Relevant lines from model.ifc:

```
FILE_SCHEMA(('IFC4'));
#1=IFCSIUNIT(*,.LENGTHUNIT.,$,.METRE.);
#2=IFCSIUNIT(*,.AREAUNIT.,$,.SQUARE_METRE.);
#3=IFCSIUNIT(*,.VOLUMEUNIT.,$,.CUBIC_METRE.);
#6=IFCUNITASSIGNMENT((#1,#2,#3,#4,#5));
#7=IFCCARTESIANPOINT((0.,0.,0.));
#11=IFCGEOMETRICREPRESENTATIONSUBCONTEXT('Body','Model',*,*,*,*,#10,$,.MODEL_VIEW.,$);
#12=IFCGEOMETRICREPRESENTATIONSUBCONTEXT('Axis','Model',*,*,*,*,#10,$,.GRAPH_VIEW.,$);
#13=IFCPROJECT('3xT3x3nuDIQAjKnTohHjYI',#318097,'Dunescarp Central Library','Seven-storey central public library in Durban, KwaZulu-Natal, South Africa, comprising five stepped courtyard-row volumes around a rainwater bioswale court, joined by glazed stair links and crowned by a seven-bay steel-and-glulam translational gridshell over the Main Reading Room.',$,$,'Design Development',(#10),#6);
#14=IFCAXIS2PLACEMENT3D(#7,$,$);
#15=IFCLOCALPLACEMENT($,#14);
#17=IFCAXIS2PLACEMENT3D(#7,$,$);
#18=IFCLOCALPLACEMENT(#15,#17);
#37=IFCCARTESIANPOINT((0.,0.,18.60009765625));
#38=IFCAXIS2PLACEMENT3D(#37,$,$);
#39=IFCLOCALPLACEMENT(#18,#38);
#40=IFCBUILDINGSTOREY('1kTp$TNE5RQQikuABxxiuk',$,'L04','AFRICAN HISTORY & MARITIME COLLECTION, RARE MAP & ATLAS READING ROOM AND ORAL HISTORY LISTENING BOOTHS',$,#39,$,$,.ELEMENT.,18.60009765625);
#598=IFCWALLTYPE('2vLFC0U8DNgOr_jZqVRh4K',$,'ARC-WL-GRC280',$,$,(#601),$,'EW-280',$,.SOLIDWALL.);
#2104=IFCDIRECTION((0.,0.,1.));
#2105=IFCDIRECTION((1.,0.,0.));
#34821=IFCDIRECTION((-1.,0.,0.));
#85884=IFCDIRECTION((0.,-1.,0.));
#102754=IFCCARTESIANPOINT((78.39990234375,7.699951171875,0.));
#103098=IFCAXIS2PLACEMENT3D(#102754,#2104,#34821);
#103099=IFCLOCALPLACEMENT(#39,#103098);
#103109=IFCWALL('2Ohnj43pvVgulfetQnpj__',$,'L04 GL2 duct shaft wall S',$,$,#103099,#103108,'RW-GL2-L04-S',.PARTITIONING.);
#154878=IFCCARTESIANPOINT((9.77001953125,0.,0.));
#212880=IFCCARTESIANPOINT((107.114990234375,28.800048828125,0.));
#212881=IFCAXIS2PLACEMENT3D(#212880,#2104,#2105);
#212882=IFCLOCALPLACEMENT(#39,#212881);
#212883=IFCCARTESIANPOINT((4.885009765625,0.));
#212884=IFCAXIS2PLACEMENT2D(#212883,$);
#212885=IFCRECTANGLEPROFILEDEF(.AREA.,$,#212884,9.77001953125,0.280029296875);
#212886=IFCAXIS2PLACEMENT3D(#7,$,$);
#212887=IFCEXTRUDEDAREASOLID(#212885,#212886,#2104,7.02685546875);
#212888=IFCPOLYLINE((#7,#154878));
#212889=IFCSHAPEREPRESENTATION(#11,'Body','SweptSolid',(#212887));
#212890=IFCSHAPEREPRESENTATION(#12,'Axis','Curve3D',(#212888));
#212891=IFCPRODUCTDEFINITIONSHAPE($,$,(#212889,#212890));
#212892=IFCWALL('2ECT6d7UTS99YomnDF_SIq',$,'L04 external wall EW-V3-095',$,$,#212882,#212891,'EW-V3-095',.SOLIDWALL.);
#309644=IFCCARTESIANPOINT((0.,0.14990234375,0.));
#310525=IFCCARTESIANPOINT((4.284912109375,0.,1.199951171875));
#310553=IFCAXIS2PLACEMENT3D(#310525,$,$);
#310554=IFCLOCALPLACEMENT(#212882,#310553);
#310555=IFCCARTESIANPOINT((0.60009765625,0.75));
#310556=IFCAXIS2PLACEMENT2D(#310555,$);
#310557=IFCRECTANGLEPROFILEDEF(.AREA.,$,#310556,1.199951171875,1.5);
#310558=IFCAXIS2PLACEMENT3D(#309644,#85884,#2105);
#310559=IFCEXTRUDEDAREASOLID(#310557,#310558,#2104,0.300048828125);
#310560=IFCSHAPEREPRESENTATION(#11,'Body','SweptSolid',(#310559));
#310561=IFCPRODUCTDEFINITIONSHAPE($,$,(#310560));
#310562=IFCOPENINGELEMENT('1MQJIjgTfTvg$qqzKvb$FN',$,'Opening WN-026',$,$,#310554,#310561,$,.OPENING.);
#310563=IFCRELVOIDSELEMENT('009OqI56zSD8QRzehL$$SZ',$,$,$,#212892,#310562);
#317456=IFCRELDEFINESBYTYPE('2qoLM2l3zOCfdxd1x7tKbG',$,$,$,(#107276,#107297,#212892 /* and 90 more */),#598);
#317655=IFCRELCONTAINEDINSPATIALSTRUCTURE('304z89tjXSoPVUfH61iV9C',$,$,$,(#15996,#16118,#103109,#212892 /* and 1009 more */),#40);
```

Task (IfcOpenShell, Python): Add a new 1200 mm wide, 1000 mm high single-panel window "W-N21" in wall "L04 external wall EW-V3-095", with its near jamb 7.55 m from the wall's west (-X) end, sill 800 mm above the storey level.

```python
import numpy as np
import ifcopenshell
import ifcopenshell.api.feature
import ifcopenshell.api.geometry
import ifcopenshell.api.root
import ifcopenshell.api.spatial
import ifcopenshell.geom
import ifcopenshell.util.element
import ifcopenshell.util.placement
import ifcopenshell.util.representation
import ifcopenshell.util.shape
import ifcopenshell.util.unit

model = ifcopenshell.open("model.ifc")
unit_scale = ifcopenshell.util.unit.calculate_unit_scale(model)
settings = ifcopenshell.geom.settings()


def volume(element):
    """Net volume in cubic metres, openings subtracted."""
    shape = ifcopenshell.geom.create_shape(settings, element)
    return ifcopenshell.util.shape.get_volume(shape.geometry)


wall = model.by_id(212892)
storey = ifcopenshell.util.element.get_container(wall, ifc_class="IfcBuildingStorey")
context = ifcopenshell.util.representation.get_context(model, "Model", "Body", "MODEL_VIEW")
before = volume(wall)

width, height, from_end, sill = 1.2, 1, 7.55, 0.8  # metres

# The wall runs along its own X axis, and the end named is its -X end.
wall_shape = ifcopenshell.geom.create_shape(settings, wall)
x, y, z = ifcopenshell.util.shape.get_vertices(wall_shape.geometry).T
start = x.min() + from_end
face, thickness = float(y.min()), float(y.max() - y.min())
wall_matrix = ifcopenshell.util.placement.get_local_placement(wall.ObjectPlacement)
level = ifcopenshell.util.placement.get_local_placement(storey.ObjectPlacement)[2, 3]


def in_wall(x, y):
    """Placement at x, y metres in the wall's axes, at sill height."""
    matrix = wall_matrix.copy()
    matrix[:, 3] = wall_matrix @ np.array([x / unit_scale, y / unit_scale, 0.0, 1.0])
    matrix[2, 3] = level + sill / unit_scale
    return matrix


# Opening: a box that overshoots both wall faces by 50 mm.
opening = ifcopenshell.api.root.create_entity(model, ifc_class="IfcOpeningElement", predefined_type="OPENING")
box = ifcopenshell.api.geometry.add_wall_representation(
    model, context=context, length=width, height=height, thickness=thickness + 0.1
)
ifcopenshell.api.geometry.assign_representation(model, product=opening, representation=box)
ifcopenshell.api.geometry.edit_object_placement(model, product=opening, matrix=in_wall(start, face - 0.05), is_si=False)
ifcopenshell.api.feature.add_feature(model, feature=opening, element=wall)

window = ifcopenshell.api.root.create_entity(model, ifc_class="IfcWindow", name="W-N21", predefined_type="WINDOW")
window.OverallWidth, window.OverallHeight = width / unit_scale, height / unit_scale
window.PartitioningType = "SINGLE_PANEL"
body = ifcopenshell.api.geometry.add_window_representation(
    model,
    context=context,
    overall_width=window.OverallWidth,
    overall_height=window.OverallHeight,
    partition_type="SINGLE_PANEL",
)
ifcopenshell.api.geometry.assign_representation(model, product=window, representation=body)
ifcopenshell.api.spatial.assign_container(model, products=[window], relating_structure=storey)
ifcopenshell.api.feature.add_filling(model, opening=opening, element=window)

# Centre the window in the wall's thickness.
ifcopenshell.api.geometry.edit_object_placement(model, product=window, matrix=in_wall(start, face), is_si=False)
window_shape = ifcopenshell.geom.create_shape(settings, window)
depth = ifcopenshell.util.shape.get_vertices(window_shape.geometry)[:, 1]
offset = face + thickness / 2 - (depth.min() + depth.max()) / 2
ifcopenshell.api.geometry.edit_object_placement(model, product=window, matrix=in_wall(start, offset), is_si=False)

after = volume(wall)

print(f"wall volume {before:.3f} -> {after:.3f} m3")

model.write("model_edited.ifc")
```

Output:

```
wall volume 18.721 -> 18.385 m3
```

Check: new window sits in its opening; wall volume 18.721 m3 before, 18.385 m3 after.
